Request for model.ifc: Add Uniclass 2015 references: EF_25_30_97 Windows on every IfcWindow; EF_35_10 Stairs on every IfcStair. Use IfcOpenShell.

First a look at what the model holds.

```python
import ifcopenshell

model = ifcopenshell.open("model.ifc")
print(model.schema)
print("classifications:", [c.Name for c in model.by_type("IfcClassification")])
for ifc_class in ("IfcDoor", "IfcRoof", "IfcStair", "IfcWall", "IfcWindow"):
    print(ifc_class, len(model.by_type(ifc_class)))
```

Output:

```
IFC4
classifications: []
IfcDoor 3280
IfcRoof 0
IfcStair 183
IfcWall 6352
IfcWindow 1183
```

```python
import ifcopenshell
import ifcopenshell.api.classification

model = ifcopenshell.open("model.ifc")

system = ifcopenshell.api.classification.add_classification(model, classification="Uniclass 2015")

codes = {
    "IfcWindow": ("EF_25_30_97", "Windows"),
    "IfcStair": ("EF_35_10", "Stairs"),
}
for ifc_class, (code, name) in codes.items():
    products = model.by_type(ifc_class)
    ifcopenshell.api.classification.add_reference(
        model, products=products, classification=system, identification=code, name=name
    )
    print(code, len(products))

model.write("model_rev.ifc")
```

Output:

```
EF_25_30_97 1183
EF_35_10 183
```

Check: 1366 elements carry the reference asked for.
